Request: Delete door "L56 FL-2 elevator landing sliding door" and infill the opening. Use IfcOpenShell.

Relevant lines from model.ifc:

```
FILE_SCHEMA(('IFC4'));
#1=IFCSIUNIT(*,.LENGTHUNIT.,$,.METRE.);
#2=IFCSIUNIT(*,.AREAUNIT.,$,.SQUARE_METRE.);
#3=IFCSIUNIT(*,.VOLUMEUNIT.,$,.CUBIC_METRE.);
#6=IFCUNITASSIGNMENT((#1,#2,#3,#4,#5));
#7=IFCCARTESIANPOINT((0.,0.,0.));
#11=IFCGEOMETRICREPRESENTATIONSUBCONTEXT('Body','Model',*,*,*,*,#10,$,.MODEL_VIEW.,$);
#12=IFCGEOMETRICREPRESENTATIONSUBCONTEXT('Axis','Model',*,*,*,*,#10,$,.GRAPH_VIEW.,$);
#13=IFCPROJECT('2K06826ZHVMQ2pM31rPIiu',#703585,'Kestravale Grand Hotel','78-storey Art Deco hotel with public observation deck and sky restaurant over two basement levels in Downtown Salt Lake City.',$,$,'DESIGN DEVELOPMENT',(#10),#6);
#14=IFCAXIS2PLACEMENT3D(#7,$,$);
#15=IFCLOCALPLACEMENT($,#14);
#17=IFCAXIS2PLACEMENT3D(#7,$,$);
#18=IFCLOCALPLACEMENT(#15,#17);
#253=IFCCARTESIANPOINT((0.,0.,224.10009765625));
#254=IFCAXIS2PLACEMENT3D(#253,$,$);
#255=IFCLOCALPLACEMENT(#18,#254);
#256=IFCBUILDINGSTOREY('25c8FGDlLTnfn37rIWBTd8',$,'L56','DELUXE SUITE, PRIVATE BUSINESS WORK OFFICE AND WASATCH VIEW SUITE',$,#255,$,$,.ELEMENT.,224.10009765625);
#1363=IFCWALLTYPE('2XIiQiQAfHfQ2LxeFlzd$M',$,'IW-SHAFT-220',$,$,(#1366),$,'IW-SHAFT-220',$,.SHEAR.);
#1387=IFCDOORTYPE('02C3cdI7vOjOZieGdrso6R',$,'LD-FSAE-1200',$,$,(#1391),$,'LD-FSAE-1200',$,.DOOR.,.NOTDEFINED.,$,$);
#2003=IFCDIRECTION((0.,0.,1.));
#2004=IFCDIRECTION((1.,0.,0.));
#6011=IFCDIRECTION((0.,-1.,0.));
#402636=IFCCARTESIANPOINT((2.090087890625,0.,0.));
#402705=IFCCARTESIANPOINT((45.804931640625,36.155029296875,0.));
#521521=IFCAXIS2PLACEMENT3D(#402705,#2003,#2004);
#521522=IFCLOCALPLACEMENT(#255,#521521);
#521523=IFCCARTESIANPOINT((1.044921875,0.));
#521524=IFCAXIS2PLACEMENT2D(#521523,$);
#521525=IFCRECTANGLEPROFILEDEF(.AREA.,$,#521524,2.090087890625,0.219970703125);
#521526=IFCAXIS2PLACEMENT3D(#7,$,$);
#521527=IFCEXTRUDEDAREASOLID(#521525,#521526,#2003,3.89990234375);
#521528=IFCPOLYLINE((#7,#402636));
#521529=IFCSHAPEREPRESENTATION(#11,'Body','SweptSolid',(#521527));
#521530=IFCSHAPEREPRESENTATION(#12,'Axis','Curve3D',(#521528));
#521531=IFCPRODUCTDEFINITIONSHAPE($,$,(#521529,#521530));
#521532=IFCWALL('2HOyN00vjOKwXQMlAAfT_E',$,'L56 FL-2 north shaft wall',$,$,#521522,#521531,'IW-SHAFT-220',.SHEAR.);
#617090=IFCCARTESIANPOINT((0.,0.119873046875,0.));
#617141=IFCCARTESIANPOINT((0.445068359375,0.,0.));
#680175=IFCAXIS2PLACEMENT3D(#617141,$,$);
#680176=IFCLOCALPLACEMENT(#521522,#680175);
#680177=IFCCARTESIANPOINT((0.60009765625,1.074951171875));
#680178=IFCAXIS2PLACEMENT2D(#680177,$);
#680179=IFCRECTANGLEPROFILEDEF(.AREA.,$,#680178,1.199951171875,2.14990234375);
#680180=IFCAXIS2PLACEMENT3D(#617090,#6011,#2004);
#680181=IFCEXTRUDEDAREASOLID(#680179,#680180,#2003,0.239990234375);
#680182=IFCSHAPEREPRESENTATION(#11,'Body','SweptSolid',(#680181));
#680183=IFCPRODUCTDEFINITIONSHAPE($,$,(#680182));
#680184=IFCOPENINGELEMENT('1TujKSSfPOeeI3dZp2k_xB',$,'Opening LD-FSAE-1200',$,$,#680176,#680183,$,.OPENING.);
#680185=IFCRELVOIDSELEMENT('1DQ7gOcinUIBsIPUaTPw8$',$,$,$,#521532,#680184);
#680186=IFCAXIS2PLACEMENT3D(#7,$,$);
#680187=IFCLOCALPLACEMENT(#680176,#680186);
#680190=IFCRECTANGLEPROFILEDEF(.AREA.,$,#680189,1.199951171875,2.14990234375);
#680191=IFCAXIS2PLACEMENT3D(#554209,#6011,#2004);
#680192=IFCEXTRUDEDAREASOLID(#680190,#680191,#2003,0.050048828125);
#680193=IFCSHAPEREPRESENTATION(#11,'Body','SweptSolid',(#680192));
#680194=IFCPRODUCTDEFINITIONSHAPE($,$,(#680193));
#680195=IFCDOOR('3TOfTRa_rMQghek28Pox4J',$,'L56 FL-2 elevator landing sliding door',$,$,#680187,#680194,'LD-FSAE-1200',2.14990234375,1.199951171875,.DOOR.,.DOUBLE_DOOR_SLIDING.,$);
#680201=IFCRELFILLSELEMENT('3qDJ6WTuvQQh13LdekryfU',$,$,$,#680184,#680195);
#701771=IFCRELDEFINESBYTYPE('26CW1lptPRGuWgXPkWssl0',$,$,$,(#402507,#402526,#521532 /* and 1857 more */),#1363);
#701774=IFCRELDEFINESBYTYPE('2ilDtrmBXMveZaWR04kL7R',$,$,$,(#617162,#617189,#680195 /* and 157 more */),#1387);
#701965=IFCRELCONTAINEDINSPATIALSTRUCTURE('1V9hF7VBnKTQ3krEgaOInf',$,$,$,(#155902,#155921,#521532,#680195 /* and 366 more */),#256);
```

```python
import ifcopenshell
import ifcopenshell.api.feature
import ifcopenshell.api.root
import ifcopenshell.geom
import ifcopenshell.util.shape

model = ifcopenshell.open("model.ifc")
settings = ifcopenshell.geom.settings()


def volume(element):
    """Net volume in cubic metres, openings subtracted."""
    shape = ifcopenshell.geom.create_shape(settings, element)
    return ifcopenshell.util.shape.get_volume(shape.geometry)


door = model.by_guid("3TOfTRa_rMQghek28Pox4J")
opening = door.FillsVoids[0].RelatingOpeningElement
wall = opening.VoidsElements[0].RelatingBuildingElement
before = volume(wall)

ifcopenshell.api.root.remove_product(model, product=door)
ifcopenshell.api.feature.remove_feature(model, feature=opening)

after = volume(wall)

print(f"wall volume {before:.3f} -> {after:.3f} m3")

model.write("model_updated.ifc")
```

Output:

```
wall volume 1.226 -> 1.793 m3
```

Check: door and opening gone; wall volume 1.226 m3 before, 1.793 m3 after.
